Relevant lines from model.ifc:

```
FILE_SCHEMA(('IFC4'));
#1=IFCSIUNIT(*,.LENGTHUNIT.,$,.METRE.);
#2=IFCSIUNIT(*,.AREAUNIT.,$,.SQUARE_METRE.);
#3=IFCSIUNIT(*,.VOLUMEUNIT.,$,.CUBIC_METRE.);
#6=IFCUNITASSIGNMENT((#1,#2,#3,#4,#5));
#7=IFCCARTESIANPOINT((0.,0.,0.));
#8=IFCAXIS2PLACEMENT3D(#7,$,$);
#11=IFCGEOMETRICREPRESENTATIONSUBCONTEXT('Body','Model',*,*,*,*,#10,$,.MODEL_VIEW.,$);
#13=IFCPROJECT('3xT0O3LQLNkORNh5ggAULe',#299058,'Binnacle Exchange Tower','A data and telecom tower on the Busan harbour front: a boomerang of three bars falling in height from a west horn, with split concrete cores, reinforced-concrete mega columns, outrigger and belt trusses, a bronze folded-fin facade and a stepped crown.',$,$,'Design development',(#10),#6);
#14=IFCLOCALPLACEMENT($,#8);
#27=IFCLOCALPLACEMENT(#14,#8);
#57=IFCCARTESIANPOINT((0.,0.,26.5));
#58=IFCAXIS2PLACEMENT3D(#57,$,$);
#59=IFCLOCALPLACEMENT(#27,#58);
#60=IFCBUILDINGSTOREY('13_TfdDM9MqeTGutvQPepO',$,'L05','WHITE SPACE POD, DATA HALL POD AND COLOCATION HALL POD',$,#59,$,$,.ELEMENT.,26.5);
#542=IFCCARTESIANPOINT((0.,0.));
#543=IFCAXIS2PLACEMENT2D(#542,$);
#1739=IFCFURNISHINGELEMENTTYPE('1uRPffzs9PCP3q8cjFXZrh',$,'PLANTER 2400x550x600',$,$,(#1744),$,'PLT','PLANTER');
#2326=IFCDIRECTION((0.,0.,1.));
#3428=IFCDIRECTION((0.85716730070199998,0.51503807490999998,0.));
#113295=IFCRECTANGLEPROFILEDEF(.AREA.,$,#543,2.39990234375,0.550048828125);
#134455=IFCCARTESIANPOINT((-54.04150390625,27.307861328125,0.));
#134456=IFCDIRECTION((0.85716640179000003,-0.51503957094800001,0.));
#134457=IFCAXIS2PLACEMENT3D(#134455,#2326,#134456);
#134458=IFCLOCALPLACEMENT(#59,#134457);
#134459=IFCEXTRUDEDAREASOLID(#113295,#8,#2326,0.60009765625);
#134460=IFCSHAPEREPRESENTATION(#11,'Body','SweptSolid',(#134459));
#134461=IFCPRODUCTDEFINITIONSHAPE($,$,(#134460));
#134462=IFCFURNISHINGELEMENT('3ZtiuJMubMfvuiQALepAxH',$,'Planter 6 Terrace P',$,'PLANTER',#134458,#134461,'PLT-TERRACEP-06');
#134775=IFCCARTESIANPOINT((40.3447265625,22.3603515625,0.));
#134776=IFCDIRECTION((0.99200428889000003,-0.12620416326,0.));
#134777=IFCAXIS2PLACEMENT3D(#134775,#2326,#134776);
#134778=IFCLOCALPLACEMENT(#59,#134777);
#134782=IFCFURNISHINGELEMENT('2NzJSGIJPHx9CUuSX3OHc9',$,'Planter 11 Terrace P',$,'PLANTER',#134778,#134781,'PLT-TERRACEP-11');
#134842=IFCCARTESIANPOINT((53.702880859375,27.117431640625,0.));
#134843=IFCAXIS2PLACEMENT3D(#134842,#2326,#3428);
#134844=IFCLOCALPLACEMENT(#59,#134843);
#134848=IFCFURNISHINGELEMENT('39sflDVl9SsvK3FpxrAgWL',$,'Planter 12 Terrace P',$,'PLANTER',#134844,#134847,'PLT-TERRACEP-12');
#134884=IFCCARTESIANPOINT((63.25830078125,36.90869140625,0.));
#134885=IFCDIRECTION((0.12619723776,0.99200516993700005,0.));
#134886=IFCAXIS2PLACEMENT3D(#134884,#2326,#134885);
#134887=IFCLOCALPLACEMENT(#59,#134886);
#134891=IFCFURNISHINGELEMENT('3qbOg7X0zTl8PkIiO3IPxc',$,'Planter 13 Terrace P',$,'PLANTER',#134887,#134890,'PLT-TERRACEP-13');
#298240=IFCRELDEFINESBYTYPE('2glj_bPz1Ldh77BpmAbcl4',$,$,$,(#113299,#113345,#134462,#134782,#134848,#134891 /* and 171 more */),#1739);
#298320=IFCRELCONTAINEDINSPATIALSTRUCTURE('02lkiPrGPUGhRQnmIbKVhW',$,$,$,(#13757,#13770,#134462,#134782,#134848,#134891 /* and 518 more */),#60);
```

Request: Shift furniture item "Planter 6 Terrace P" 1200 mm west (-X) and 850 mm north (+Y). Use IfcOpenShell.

```python
import ifcopenshell
import ifcopenshell.api.geometry
import ifcopenshell.util.placement

model = ifcopenshell.open("model.ifc")

item = model.by_guid("3ZtiuJMubMfvuiQALepAxH")
matrix = ifcopenshell.util.placement.get_local_placement(item.ObjectPlacement)
matrix[0, 3] -= 1.2
matrix[1, 3] += 0.85
ifcopenshell.api.geometry.edit_object_placement(model, product=item, matrix=matrix, is_si=False)

print(ifcopenshell.util.placement.get_local_placement(item.ObjectPlacement).round(3) + 0.0)

model.write("model_rev.ifc")
```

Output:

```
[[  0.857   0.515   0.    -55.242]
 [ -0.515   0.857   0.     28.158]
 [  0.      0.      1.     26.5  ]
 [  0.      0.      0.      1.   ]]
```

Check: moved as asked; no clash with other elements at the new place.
